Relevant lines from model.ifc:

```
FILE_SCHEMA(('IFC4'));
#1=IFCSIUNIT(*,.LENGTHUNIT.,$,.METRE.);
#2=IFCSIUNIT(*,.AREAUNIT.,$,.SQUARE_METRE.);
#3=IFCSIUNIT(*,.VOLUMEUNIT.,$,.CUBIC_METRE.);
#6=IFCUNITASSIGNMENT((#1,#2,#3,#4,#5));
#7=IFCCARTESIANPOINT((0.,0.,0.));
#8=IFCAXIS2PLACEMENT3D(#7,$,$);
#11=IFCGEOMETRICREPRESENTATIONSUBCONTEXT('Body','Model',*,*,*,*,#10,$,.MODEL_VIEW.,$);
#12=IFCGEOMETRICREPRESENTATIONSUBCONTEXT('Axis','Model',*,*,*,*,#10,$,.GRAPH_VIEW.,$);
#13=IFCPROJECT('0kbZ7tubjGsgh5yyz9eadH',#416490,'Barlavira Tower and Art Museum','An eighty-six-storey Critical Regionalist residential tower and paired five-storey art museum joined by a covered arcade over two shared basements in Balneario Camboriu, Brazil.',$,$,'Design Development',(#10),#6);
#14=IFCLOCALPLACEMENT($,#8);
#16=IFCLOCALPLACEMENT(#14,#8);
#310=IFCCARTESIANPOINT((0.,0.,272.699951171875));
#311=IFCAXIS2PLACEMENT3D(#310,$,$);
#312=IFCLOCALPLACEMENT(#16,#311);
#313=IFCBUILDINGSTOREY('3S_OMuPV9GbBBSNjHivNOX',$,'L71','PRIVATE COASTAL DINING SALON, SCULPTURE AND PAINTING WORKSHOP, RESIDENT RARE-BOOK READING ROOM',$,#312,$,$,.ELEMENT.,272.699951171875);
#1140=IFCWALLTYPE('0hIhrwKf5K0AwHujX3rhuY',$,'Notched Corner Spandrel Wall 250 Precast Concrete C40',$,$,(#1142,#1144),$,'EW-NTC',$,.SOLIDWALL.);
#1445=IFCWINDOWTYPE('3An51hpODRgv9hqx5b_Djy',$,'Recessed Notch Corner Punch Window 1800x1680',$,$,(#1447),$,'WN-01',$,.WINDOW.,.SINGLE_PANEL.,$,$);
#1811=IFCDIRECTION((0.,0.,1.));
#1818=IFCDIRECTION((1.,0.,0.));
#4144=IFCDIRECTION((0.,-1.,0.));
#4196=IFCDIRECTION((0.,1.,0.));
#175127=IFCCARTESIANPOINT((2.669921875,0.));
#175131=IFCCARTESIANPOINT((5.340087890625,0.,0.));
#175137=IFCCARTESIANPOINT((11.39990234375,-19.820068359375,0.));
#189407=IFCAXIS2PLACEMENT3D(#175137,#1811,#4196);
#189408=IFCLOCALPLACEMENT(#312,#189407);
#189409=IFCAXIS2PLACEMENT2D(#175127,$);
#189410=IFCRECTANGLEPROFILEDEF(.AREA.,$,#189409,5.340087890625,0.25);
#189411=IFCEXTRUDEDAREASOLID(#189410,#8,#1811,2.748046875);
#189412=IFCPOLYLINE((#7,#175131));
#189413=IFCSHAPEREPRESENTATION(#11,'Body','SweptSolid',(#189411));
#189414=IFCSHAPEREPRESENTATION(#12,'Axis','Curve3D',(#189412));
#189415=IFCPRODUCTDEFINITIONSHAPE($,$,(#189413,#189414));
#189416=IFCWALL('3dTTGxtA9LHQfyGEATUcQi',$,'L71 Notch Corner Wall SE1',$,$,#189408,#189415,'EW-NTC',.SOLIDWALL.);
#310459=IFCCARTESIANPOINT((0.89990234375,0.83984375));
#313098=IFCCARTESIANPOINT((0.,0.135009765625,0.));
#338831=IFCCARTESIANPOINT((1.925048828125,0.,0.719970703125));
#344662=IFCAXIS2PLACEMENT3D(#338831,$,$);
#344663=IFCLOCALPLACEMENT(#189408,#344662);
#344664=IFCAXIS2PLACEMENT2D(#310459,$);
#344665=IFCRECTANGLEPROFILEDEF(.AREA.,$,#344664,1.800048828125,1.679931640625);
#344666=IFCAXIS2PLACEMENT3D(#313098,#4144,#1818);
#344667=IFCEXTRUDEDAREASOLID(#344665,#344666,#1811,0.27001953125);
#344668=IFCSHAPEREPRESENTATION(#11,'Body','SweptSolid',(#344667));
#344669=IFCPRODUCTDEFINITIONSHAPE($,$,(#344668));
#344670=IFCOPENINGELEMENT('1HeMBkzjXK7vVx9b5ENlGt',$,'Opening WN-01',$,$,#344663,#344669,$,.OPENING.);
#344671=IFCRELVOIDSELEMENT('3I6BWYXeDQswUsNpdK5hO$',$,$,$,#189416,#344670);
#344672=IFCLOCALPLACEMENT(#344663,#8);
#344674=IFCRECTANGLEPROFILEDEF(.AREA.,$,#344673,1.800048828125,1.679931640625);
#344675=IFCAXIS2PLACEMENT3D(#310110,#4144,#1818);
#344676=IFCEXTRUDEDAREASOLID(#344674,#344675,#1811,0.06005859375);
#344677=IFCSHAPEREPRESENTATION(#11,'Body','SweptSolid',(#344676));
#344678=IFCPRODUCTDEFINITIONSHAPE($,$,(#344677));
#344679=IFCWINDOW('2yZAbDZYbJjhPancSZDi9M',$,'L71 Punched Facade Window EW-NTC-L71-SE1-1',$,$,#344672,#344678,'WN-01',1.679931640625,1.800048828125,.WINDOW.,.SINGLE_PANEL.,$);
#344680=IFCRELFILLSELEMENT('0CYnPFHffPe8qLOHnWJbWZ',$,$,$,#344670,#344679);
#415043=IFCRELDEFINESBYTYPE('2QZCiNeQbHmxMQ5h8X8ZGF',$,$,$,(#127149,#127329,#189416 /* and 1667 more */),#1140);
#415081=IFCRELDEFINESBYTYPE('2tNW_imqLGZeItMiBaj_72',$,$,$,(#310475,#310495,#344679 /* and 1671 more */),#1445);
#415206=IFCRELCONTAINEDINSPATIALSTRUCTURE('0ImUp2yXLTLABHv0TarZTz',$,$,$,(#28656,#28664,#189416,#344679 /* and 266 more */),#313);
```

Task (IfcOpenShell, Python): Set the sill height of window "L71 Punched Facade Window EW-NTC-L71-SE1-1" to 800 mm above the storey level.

```python
import numpy as np
import ifcopenshell
import ifcopenshell.api.geometry
import ifcopenshell.geom
import ifcopenshell.util.element
import ifcopenshell.util.placement
import ifcopenshell.util.shape
import ifcopenshell.util.unit

model = ifcopenshell.open("model.ifc")
unit_scale = ifcopenshell.util.unit.calculate_unit_scale(model)

window = model.by_id(344679)
opening = window.FillsVoids[0].RelatingOpeningElement
storey = ifcopenshell.util.element.get_container(window, ifc_class="IfcBuildingStorey")
level = ifcopenshell.util.placement.get_local_placement(storey.ObjectPlacement)[2, 3]

# The opening's origin need not be at the sill, so measure its lowest point.
shape = ifcopenshell.geom.create_shape(ifcopenshell.geom.settings(), opening)
bottom = ifcopenshell.util.shape.get_shape_bottom_elevation(shape, shape.geometry) / unit_scale
dz = level + 0.8 / unit_scale - bottom

shift = np.array([0.0, 0.0, dz])
# The window is placed relative to its opening, so it follows when the opening moves.
matrix = ifcopenshell.util.placement.get_local_placement(opening.ObjectPlacement)
matrix[:3, 3] += shift
ifcopenshell.api.geometry.edit_object_placement(
    model, product=opening, matrix=matrix, is_si=False, should_transform_children=True
)

print(f"moved by {dz * unit_scale:+.3f} m")

model.write("model_updated.ifc")
```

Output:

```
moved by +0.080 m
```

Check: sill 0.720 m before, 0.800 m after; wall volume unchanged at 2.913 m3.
